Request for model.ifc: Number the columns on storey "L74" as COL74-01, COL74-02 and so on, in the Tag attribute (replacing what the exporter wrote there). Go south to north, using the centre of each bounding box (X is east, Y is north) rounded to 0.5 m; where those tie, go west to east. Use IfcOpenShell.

First a look at what the model holds.

```python
import ifcopenshell
import ifcopenshell.util.element
import ifcopenshell.util.placement

model = ifcopenshell.open("model.ifc")
print(model.schema)
storey = next(s for s in model.by_type("IfcBuildingStorey") if s.Name == "L74")
columns = [e for e in ifcopenshell.util.element.get_decomposition(storey) if e.is_a("IfcColumn")]
for e in sorted(columns, key=lambda e: e.id()):
    origin = ifcopenshell.util.placement.get_local_placement(e.ObjectPlacement)[:3, 3]
    print(e.id(), e.Tag, e.Name, origin.round(2) + 0.0, sep=" | ")
```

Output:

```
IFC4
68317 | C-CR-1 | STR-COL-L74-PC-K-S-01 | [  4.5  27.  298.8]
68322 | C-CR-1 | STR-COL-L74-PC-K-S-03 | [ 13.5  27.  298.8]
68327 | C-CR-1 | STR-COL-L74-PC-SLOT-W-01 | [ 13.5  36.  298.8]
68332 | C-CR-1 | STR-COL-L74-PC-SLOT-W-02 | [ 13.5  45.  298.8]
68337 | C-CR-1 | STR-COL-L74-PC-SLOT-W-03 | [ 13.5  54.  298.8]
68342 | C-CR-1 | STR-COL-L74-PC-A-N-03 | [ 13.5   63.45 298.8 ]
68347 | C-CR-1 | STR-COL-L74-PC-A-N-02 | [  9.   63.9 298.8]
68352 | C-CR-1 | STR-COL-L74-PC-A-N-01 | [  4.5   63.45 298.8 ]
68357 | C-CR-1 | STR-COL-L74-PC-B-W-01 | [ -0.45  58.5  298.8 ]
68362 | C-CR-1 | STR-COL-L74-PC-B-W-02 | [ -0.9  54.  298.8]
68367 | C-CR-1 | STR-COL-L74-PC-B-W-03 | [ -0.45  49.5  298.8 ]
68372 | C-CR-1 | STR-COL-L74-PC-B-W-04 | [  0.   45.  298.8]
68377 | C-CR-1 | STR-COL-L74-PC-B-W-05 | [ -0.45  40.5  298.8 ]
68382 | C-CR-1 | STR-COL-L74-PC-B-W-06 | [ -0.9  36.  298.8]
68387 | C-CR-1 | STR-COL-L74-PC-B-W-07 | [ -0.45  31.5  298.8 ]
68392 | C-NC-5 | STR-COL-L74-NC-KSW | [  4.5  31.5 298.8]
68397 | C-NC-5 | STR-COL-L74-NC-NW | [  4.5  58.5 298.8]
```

```python
import ifcopenshell
import ifcopenshell.geom
import ifcopenshell.util.element
import ifcopenshell.util.shape

model = ifcopenshell.open("model.ifc")
settings = ifcopenshell.geom.settings()
settings.set("use-world-coords", True)


def centre(element):
    shape = ifcopenshell.geom.create_shape(settings, element)
    return ifcopenshell.util.shape.get_bbox_centroid(shape.geometry)


storey = next(s for s in model.by_type("IfcBuildingStorey") if s.Name == "L74")
columns = [e for e in ifcopenshell.util.element.get_decomposition(storey) if e.is_a("IfcColumn")]

# Insertion points can sit at a corner or the storey origin, so sort by the geometry (in metres).
centres = {e: centre(e) for e in columns}
columns.sort(key=lambda e: (round(centres[e][1] / 0.5), centres[e][0]))

for i, e in enumerate(columns, start=1):
    number = f"COL74-{i:02d}"
    e.Tag = number
    print(e.id(), number)

model.write("model_rev.ifc")
```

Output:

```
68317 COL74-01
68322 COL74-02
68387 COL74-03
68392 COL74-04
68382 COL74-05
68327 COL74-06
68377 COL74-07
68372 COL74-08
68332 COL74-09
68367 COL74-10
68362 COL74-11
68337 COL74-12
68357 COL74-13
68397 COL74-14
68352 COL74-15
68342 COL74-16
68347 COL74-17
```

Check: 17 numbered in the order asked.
